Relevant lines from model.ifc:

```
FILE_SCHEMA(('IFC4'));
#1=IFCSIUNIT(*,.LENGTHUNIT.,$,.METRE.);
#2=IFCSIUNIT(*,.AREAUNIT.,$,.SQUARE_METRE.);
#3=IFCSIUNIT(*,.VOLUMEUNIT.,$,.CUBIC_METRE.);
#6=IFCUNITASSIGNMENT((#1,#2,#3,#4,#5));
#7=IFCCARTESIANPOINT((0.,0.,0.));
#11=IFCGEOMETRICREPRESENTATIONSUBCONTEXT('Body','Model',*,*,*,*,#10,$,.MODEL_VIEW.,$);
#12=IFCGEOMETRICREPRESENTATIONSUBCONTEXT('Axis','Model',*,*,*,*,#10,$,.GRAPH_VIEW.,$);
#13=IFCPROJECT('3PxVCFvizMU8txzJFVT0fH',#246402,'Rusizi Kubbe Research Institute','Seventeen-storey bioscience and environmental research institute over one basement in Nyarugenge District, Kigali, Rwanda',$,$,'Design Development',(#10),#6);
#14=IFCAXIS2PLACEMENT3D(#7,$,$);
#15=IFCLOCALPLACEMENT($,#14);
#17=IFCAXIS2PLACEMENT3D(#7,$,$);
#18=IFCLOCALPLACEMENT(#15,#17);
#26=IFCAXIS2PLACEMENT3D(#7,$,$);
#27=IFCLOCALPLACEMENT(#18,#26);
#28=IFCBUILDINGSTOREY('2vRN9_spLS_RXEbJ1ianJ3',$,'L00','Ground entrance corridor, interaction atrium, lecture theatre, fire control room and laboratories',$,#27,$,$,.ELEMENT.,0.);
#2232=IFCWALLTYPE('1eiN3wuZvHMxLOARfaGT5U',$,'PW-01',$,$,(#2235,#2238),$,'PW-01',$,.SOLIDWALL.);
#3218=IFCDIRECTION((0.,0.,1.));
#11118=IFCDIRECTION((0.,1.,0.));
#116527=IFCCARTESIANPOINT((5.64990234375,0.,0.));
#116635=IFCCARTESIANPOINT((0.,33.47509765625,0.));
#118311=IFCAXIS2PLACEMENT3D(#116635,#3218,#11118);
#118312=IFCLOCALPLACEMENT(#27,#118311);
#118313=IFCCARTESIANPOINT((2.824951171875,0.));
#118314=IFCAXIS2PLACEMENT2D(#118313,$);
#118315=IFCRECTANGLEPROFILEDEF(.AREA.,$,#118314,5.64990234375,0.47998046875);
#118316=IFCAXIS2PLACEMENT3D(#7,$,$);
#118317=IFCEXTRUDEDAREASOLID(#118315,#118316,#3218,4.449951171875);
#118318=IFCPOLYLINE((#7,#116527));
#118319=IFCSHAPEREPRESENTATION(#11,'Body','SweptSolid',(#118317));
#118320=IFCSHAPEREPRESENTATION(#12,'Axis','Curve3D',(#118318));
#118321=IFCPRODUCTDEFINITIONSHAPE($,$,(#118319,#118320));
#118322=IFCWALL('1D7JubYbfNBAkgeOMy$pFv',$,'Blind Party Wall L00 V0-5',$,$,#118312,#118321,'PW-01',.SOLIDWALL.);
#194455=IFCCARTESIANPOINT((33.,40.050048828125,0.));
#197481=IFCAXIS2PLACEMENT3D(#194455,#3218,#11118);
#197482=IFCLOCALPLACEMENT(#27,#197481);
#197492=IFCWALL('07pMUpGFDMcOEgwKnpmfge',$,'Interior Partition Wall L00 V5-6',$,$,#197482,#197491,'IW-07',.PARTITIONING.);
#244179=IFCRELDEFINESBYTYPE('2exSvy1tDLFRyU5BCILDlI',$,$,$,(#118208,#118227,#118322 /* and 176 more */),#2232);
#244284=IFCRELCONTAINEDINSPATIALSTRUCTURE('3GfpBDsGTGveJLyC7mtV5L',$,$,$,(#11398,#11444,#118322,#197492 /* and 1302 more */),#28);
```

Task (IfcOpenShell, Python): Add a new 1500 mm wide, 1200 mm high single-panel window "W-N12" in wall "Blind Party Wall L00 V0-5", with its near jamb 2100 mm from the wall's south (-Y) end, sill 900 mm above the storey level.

```python
import numpy as np
import ifcopenshell
import ifcopenshell.api.feature
import ifcopenshell.api.geometry
import ifcopenshell.api.root
import ifcopenshell.api.spatial
import ifcopenshell.geom
import ifcopenshell.util.element
import ifcopenshell.util.placement
import ifcopenshell.util.representation
import ifcopenshell.util.shape
import ifcopenshell.util.unit

model = ifcopenshell.open("model.ifc")
unit_scale = ifcopenshell.util.unit.calculate_unit_scale(model)
settings = ifcopenshell.geom.settings()


def volume(element):
    """Net volume in cubic metres, openings subtracted."""
    shape = ifcopenshell.geom.create_shape(settings, element)
    return ifcopenshell.util.shape.get_volume(shape.geometry)


wall = model.by_guid("1D7JubYbfNBAkgeOMy$pFv")
storey = ifcopenshell.util.element.get_container(wall, ifc_class="IfcBuildingStorey")
context = ifcopenshell.util.representation.get_context(model, "Model", "Body", "MODEL_VIEW")
before = volume(wall)

width, height, from_end, sill = 1.5, 1.2, 2.1, 0.9  # metres

# The wall runs along its own X axis, and the end named is its -X end.
wall_shape = ifcopenshell.geom.create_shape(settings, wall)
x, y, z = ifcopenshell.util.shape.get_vertices(wall_shape.geometry).T
start = x.min() + from_end
face, thickness = float(y.min()), float(y.max() - y.min())
wall_matrix = ifcopenshell.util.placement.get_local_placement(wall.ObjectPlacement)
level = ifcopenshell.util.placement.get_local_placement(storey.ObjectPlacement)[2, 3]


def in_wall(x, y):
    """Placement at x, y metres in the wall's axes, at sill height."""
    matrix = wall_matrix.copy()
    matrix[:, 3] = wall_matrix @ np.array([x / unit_scale, y / unit_scale, 0.0, 1.0])
    matrix[2, 3] = level + sill / unit_scale
    return matrix


# Opening: a box that overshoots both wall faces by 50 mm.
opening = ifcopenshell.api.root.create_entity(model, ifc_class="IfcOpeningElement", predefined_type="OPENING")
box = ifcopenshell.api.geometry.add_wall_representation(
    model, context=context, length=width, height=height, thickness=thickness + 0.1
)
ifcopenshell.api.geometry.assign_representation(model, product=opening, representation=box)
ifcopenshell.api.geometry.edit_object_placement(model, product=opening, matrix=in_wall(start, face - 0.05), is_si=False)
ifcopenshell.api.feature.add_feature(model, feature=opening, element=wall)

window = ifcopenshell.api.root.create_entity(model, ifc_class="IfcWindow", name="W-N12", predefined_type="WINDOW")
window.OverallWidth, window.OverallHeight = width / unit_scale, height / unit_scale
window.PartitioningType = "SINGLE_PANEL"
body = ifcopenshell.api.geometry.add_window_representation(
    model,
    context=context,
    overall_width=window.OverallWidth,
    overall_height=window.OverallHeight,
    partition_type="SINGLE_PANEL",
)
ifcopenshell.api.geometry.assign_representation(model, product=window, representation=body)
ifcopenshell.api.spatial.assign_container(model, products=[window], relating_structure=storey)
ifcopenshell.api.feature.add_filling(model, opening=opening, element=window)

# Centre the window in the wall's thickness.
ifcopenshell.api.geometry.edit_object_placement(model, product=window, matrix=in_wall(start, face), is_si=False)
window_shape = ifcopenshell.geom.create_shape(settings, window)
depth = ifcopenshell.util.shape.get_vertices(window_shape.geometry)[:, 1]
offset = face + thickness / 2 - (depth.min() + depth.max()) / 2
ifcopenshell.api.geometry.edit_object_placement(model, product=window, matrix=in_wall(start, offset), is_si=False)

after = volume(wall)

print(f"wall volume {before:.3f} -> {after:.3f} m3")

model.write("model_rev.ifc")
```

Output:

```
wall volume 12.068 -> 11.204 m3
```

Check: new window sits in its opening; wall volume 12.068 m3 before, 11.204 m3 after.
